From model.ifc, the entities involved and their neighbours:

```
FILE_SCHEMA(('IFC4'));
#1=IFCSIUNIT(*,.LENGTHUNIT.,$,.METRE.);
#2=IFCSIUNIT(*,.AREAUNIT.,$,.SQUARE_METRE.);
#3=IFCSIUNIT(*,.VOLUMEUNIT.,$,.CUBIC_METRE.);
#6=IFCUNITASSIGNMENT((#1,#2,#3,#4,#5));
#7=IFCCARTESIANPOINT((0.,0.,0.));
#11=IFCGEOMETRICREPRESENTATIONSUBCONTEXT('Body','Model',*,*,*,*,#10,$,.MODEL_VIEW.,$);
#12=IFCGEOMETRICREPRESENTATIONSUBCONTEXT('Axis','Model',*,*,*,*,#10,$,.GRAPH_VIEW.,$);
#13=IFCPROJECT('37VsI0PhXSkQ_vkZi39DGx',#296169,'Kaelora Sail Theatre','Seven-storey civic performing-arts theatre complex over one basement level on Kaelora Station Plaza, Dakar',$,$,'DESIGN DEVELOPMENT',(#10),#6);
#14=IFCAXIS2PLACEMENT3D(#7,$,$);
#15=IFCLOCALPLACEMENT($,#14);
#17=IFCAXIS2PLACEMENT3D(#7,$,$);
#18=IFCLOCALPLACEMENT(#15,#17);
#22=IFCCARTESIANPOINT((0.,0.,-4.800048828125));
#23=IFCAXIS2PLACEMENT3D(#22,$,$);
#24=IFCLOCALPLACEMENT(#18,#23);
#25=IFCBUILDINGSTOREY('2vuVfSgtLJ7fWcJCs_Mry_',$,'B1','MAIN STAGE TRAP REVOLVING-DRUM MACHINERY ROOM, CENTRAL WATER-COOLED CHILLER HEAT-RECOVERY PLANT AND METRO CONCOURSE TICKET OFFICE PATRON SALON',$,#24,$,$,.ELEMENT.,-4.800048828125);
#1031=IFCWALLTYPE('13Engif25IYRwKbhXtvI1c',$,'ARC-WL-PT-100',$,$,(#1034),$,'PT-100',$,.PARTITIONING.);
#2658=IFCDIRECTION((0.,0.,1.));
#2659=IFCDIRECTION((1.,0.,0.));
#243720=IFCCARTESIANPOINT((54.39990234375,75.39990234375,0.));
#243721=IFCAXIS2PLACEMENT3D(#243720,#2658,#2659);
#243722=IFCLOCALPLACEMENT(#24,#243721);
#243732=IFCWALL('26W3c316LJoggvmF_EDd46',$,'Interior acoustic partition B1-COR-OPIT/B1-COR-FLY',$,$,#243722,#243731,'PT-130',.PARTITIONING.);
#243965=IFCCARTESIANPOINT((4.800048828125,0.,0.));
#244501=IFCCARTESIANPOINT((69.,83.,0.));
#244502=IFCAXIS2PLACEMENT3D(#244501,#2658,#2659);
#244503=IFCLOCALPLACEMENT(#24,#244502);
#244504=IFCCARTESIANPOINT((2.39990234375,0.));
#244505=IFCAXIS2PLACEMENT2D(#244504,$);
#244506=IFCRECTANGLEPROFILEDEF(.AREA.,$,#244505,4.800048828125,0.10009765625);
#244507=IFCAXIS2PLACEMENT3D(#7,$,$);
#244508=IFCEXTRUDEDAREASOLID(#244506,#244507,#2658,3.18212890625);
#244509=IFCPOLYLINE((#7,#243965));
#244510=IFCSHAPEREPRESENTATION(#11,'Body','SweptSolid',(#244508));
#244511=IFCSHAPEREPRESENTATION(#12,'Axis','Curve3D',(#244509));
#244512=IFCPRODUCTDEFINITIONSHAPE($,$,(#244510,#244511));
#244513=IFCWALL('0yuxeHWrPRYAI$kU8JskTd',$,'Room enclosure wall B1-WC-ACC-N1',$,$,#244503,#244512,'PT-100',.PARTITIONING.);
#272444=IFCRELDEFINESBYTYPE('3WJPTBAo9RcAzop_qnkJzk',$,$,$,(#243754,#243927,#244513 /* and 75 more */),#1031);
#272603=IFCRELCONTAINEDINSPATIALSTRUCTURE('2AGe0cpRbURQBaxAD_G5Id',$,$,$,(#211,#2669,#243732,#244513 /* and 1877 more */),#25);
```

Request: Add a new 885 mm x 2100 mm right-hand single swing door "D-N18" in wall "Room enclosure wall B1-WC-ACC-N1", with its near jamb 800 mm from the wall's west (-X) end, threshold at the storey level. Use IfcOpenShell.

```python
import numpy as np
import ifcopenshell
import ifcopenshell.api.feature
import ifcopenshell.api.geometry
import ifcopenshell.api.root
import ifcopenshell.api.spatial
import ifcopenshell.geom
import ifcopenshell.util.element
import ifcopenshell.util.placement
import ifcopenshell.util.representation
import ifcopenshell.util.shape
import ifcopenshell.util.unit

model = ifcopenshell.open("model.ifc")
unit_scale = ifcopenshell.util.unit.calculate_unit_scale(model)
settings = ifcopenshell.geom.settings()


def volume(element):
    """Net volume in cubic metres, openings subtracted."""
    shape = ifcopenshell.geom.create_shape(settings, element)
    return ifcopenshell.util.shape.get_volume(shape.geometry)


wall = model.by_guid("0yuxeHWrPRYAI$kU8JskTd")
storey = ifcopenshell.util.element.get_container(wall, ifc_class="IfcBuildingStorey")
context = ifcopenshell.util.representation.get_context(model, "Model", "Body", "MODEL_VIEW")
before = volume(wall)

width, height, from_end, sill = 0.885, 2.1, 0.8, 0.0  # metres

# The wall runs along its own X axis, and the end named is its -X end.
wall_shape = ifcopenshell.geom.create_shape(settings, wall)
x, y, z = ifcopenshell.util.shape.get_vertices(wall_shape.geometry).T
start = x.min() + from_end
face, thickness = float(y.min()), float(y.max() - y.min())
wall_matrix = ifcopenshell.util.placement.get_local_placement(wall.ObjectPlacement)
level = ifcopenshell.util.placement.get_local_placement(storey.ObjectPlacement)[2, 3]


def in_wall(x, y):
    """Placement at x, y metres in the wall's axes, at sill height."""
    matrix = wall_matrix.copy()
    matrix[:, 3] = wall_matrix @ np.array([x / unit_scale, y / unit_scale, 0.0, 1.0])
    matrix[2, 3] = level + sill / unit_scale
    return matrix


# Opening: a box that overshoots both wall faces by 50 mm.
opening = ifcopenshell.api.root.create_entity(model, ifc_class="IfcOpeningElement", predefined_type="OPENING")
box = ifcopenshell.api.geometry.add_wall_representation(
    model, context=context, length=width, height=height, thickness=thickness + 0.1
)
ifcopenshell.api.geometry.assign_representation(model, product=opening, representation=box)
ifcopenshell.api.geometry.edit_object_placement(model, product=opening, matrix=in_wall(start, face - 0.05), is_si=False)
ifcopenshell.api.feature.add_feature(model, feature=opening, element=wall)

door = ifcopenshell.api.root.create_entity(model, ifc_class="IfcDoor", name="D-N18", predefined_type="DOOR")
door.OverallWidth, door.OverallHeight = width / unit_scale, height / unit_scale
door.OperationType = "SINGLE_SWING_RIGHT"
body = ifcopenshell.api.geometry.add_door_representation(
    model,
    context=context,
    overall_width=door.OverallWidth,
    overall_height=door.OverallHeight,
    operation_type="SINGLE_SWING_RIGHT",
    lining_properties={"LiningDepth": thickness / unit_scale, "ThresholdDepth": thickness / unit_scale},
)
ifcopenshell.api.geometry.assign_representation(model, product=door, representation=body)
ifcopenshell.api.spatial.assign_container(model, products=[door], relating_structure=storey)
ifcopenshell.api.feature.add_filling(model, opening=opening, element=door)

# The lining spans the wall, so the door starts at the wall face.
ifcopenshell.api.geometry.edit_object_placement(model, product=door, matrix=in_wall(start, face), is_si=False)

after = volume(wall)

print(f"wall volume {before:.3f} -> {after:.3f} m3")

model.write("model_updated.ifc")
```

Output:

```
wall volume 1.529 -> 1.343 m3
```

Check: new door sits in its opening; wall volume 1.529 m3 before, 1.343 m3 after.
